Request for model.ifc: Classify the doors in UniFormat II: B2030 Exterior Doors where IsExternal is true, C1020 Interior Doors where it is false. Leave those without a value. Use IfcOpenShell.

First a look at what the model holds.

```python
import ifcopenshell
import ifcopenshell.util.element

model = ifcopenshell.open("model.ifc")
print(model.schema)
print("classifications:", [c.Name for c in model.by_type("IfcClassification")])
values = [ifcopenshell.util.element.get_pset(e, "Pset_DoorCommon", "IsExternal") for e in model.by_type("IfcDoor")]
for value in (True, False, None):
    print("IsExternal", value, values.count(value))
```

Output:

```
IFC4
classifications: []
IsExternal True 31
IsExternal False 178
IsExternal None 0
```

```python
import ifcopenshell
import ifcopenshell.api.classification
import ifcopenshell.util.element

model = ifcopenshell.open("model.ifc")

system = ifcopenshell.api.classification.add_classification(model, classification="UniFormat II")

doors = model.by_type("IfcDoor")
external = {e: ifcopenshell.util.element.get_pset(e, "Pset_DoorCommon", "IsExternal") for e in doors}
for flag, code, name in ((True, "B2030", "Exterior Doors"), (False, "C1020", "Interior Doors")):
    products = [e for e in doors if external[e] is flag]
    ifcopenshell.api.classification.add_reference(
        model, products=products, classification=system, identification=code, name=name
    )
    print(code, len(products))

model.write("model_rev.ifc")
```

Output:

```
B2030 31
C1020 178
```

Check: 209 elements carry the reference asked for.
